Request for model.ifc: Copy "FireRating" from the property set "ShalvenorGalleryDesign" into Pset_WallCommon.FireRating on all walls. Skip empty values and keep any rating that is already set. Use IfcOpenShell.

First a look at what the model holds.

```python
import ifcopenshell
import ifcopenshell.util.element

model = ifcopenshell.open("model.ifc")
print(model.schema)
walls = model.by_type("IfcWall")
print(len(walls), "walls")
for e in walls[:8]:
    source = ifcopenshell.util.element.get_pset(e, "ShalvenorGalleryDesign", "FireRating")
    target = ifcopenshell.util.element.get_pset(e, "Pset_WallCommon", "FireRating")
    print(e.id(), repr(source), repr(target), sep=" | ")
```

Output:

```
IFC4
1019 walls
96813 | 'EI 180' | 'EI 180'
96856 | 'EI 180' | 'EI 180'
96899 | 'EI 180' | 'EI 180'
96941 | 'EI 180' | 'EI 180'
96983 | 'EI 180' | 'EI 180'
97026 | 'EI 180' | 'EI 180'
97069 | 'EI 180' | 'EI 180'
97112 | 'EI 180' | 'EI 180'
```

```python
import ifcopenshell
import ifcopenshell.api.pset
import ifcopenshell.util.element

model = ifcopenshell.open("model.ifc")

count = 0
for e in model.by_type("IfcWall"):
    value = ifcopenshell.util.element.get_pset(e, "ShalvenorGalleryDesign", "FireRating")
    current = ifcopenshell.util.element.get_pset(e, "Pset_WallCommon", "FireRating")
    if not value or not value.strip() or current:
        continue
    # add_pset returns the element's existing set when there is one.
    pset = ifcopenshell.api.pset.add_pset(model, product=e, name="Pset_WallCommon")
    ifcopenshell.api.pset.edit_pset(model, pset=pset, properties={"FireRating": value})
    count += 1

print(count, "walls updated")

model.write("model_edited.ifc")
```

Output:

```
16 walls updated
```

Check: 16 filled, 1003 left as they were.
